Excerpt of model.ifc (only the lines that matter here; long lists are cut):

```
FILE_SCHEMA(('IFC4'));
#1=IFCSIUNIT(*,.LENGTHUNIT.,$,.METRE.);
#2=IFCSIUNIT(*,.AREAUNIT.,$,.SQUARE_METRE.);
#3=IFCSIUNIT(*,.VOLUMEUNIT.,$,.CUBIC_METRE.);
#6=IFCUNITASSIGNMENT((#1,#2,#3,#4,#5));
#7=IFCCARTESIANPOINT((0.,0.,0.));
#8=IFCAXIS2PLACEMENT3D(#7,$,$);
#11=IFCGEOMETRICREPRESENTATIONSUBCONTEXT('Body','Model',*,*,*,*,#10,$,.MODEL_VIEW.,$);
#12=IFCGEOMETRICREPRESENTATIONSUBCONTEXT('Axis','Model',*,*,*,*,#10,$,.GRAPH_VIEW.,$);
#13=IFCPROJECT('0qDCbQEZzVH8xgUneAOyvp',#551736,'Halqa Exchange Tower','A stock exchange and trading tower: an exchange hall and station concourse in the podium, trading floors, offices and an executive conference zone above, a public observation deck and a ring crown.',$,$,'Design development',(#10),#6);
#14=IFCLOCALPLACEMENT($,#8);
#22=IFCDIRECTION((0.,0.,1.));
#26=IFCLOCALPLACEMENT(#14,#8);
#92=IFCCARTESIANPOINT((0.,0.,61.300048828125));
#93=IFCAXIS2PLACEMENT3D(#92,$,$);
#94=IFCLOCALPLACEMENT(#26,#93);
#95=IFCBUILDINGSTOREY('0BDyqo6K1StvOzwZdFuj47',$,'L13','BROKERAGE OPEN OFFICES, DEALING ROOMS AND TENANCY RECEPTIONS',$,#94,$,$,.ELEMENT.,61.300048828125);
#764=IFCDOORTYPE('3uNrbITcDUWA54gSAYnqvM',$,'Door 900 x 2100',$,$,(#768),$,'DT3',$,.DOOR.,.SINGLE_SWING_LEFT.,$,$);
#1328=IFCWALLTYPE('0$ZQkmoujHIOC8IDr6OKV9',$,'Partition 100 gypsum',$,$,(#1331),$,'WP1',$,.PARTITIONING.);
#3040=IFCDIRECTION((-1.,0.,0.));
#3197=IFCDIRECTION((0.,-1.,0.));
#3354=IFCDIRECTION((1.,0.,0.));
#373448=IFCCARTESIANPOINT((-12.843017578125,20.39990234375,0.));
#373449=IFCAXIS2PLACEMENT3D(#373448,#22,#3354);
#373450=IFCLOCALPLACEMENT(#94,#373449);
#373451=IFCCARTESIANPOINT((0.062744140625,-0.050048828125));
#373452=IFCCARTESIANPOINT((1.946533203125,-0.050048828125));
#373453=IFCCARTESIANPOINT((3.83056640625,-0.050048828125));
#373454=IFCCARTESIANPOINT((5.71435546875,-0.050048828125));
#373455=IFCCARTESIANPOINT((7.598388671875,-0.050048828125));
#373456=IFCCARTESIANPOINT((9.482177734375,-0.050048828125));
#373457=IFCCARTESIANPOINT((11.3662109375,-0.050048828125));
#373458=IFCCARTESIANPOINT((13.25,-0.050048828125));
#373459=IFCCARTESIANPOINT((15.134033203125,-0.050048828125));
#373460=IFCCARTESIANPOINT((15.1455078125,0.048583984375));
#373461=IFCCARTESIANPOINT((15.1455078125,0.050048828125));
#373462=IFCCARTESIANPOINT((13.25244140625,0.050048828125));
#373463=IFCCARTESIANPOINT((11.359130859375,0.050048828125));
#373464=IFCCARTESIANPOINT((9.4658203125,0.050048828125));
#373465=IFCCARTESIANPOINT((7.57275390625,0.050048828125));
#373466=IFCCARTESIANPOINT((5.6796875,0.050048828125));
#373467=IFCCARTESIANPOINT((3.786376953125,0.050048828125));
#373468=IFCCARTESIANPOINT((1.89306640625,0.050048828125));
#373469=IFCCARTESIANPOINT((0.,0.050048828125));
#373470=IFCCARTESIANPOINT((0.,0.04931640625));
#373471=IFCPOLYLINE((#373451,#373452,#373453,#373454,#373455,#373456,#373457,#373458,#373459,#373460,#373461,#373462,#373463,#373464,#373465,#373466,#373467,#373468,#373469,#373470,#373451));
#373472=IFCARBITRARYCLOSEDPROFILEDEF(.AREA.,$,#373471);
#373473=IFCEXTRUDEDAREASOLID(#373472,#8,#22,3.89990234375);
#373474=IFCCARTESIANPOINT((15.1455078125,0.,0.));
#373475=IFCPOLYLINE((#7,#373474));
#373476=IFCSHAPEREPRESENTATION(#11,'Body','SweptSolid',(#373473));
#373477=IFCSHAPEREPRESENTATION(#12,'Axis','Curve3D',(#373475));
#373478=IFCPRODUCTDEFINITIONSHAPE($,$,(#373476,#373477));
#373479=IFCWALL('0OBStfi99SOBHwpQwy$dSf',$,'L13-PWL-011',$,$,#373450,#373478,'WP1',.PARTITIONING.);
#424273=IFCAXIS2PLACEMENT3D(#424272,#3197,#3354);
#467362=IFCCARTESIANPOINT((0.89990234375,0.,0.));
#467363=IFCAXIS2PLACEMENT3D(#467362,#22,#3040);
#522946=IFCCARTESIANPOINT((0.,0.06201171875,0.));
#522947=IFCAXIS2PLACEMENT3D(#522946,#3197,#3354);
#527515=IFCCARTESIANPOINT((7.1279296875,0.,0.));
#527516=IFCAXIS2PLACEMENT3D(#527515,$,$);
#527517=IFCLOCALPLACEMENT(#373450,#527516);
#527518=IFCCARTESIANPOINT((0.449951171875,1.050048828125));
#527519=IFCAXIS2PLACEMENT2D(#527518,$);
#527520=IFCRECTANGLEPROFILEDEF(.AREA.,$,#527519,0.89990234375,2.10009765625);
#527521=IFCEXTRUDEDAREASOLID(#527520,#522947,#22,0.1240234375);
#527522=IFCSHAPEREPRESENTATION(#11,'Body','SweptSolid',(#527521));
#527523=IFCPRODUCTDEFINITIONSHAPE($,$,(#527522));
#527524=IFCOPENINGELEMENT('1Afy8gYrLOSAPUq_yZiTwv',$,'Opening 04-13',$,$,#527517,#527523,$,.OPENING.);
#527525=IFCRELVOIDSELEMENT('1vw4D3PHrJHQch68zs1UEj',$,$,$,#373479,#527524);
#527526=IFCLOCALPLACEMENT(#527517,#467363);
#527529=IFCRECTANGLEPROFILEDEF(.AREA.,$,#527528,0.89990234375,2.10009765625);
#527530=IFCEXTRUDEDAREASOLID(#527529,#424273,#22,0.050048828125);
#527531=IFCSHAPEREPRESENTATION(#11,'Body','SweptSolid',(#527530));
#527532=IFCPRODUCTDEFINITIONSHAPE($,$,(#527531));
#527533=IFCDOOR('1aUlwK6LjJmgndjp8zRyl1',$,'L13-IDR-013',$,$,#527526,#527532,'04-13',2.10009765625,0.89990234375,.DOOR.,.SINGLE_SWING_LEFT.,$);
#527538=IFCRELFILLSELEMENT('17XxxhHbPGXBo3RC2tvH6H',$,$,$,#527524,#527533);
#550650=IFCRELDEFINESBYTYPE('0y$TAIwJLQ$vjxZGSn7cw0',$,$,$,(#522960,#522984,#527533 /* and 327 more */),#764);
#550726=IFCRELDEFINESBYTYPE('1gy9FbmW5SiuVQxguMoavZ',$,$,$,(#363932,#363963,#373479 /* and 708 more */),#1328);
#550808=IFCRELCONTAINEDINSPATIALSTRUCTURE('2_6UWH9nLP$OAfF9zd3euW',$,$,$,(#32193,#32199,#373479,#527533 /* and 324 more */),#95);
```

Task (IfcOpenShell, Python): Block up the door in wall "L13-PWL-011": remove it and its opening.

```python
import ifcopenshell
import ifcopenshell.api.feature
import ifcopenshell.api.root
import ifcopenshell.geom
import ifcopenshell.util.shape

model = ifcopenshell.open("model.ifc")
settings = ifcopenshell.geom.settings()


def volume(element):
    """Net volume in cubic metres, openings subtracted."""
    shape = ifcopenshell.geom.create_shape(settings, element)
    return ifcopenshell.util.shape.get_volume(shape.geometry)


door = model.by_guid("1aUlwK6LjJmgndjp8zRyl1")
opening = door.FillsVoids[0].RelatingOpeningElement
wall = opening.VoidsElements[0].RelatingBuildingElement
before = volume(wall)

ifcopenshell.api.root.remove_product(model, product=door)
ifcopenshell.api.feature.remove_feature(model, feature=opening)

after = volume(wall)

print(f"wall volume {before:.3f} -> {after:.3f} m3")

model.write("model-out.ifc")
```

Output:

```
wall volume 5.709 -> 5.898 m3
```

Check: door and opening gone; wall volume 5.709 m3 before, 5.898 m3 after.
